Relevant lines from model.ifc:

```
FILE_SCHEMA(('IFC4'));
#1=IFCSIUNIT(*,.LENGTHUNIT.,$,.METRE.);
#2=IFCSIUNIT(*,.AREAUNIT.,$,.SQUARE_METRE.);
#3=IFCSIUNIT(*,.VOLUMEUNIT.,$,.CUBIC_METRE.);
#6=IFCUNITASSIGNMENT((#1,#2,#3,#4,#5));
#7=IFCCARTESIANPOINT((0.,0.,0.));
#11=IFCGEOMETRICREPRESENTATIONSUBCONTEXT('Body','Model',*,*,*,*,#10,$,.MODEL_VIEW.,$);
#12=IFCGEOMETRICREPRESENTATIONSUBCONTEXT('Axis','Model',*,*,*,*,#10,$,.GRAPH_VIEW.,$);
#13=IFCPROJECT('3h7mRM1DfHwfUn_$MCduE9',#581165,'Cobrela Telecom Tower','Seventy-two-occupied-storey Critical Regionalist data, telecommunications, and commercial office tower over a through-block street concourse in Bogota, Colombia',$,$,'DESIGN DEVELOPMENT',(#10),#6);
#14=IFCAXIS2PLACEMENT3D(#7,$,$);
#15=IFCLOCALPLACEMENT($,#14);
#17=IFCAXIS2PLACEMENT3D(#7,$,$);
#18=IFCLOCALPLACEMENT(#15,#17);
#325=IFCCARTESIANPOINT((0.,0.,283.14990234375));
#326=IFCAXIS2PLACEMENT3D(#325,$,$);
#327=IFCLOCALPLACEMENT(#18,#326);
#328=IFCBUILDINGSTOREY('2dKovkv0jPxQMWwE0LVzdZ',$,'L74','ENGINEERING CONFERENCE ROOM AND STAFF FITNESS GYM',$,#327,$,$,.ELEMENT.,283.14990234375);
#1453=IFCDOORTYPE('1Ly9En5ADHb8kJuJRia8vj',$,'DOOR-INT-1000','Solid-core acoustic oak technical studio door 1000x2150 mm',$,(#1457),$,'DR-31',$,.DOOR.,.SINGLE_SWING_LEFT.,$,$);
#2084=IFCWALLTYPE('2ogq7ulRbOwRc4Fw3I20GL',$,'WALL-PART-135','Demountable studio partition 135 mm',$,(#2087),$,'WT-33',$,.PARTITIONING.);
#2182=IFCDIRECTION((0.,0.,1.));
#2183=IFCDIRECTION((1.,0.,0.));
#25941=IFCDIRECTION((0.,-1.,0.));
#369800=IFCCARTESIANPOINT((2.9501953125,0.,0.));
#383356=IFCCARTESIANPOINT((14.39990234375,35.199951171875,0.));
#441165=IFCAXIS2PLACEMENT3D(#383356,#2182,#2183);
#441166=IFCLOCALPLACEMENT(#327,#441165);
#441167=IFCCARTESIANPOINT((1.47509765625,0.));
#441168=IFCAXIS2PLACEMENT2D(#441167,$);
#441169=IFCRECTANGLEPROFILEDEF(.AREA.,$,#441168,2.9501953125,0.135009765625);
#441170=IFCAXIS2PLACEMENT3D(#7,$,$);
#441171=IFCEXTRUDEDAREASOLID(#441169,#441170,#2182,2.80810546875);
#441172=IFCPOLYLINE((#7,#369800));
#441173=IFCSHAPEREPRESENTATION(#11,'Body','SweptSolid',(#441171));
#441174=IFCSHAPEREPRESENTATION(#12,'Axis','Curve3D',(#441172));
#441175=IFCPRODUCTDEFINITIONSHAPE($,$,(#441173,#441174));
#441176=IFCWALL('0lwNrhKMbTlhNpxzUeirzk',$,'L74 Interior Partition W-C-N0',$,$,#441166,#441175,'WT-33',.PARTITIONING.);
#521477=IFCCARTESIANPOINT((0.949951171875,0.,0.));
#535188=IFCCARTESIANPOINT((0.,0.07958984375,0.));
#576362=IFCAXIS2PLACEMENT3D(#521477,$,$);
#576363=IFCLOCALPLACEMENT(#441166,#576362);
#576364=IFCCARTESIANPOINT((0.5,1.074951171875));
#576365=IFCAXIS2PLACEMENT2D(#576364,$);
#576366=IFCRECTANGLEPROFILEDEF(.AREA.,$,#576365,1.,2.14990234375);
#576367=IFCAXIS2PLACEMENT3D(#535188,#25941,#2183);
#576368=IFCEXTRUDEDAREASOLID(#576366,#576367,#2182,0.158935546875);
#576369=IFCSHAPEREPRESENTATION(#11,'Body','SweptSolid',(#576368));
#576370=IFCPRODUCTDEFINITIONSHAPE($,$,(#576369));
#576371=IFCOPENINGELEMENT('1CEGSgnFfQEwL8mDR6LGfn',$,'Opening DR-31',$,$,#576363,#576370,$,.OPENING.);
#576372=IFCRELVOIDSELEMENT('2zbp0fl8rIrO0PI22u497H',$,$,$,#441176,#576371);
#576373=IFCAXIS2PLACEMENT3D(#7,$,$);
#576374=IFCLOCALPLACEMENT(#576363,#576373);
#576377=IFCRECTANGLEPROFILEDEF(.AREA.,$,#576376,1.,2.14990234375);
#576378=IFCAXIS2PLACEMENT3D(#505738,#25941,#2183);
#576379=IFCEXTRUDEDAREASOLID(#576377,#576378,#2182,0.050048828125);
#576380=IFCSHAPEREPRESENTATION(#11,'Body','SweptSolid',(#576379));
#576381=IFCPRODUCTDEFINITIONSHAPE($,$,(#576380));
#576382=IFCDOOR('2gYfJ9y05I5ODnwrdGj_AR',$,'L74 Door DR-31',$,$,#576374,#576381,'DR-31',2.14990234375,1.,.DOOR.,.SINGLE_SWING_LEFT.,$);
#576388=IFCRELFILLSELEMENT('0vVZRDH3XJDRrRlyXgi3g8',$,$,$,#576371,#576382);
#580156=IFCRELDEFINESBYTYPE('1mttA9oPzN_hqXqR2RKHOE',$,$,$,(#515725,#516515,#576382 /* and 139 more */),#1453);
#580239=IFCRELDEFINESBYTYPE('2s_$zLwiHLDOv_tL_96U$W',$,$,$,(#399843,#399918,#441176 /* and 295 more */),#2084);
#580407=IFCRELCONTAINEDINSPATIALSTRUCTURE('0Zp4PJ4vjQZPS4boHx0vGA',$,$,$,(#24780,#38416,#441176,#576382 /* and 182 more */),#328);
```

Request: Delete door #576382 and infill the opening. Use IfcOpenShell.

```python
import ifcopenshell
import ifcopenshell.api.feature
import ifcopenshell.api.root
import ifcopenshell.geom
import ifcopenshell.util.shape

model = ifcopenshell.open("model.ifc")
settings = ifcopenshell.geom.settings()


def volume(element):
    """Net volume in cubic metres, openings subtracted."""
    shape = ifcopenshell.geom.create_shape(settings, element)
    return ifcopenshell.util.shape.get_volume(shape.geometry)


door = model.by_guid("2gYfJ9y05I5ODnwrdGj_AR")
opening = door.FillsVoids[0].RelatingOpeningElement
wall = opening.VoidsElements[0].RelatingBuildingElement
before = volume(wall)

ifcopenshell.api.root.remove_product(model, product=door)
ifcopenshell.api.feature.remove_feature(model, feature=opening)

after = volume(wall)

print(f"wall volume {before:.3f} -> {after:.3f} m3")

model.write("model_rev.ifc")
```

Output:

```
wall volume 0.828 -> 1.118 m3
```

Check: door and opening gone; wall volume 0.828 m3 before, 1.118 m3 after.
